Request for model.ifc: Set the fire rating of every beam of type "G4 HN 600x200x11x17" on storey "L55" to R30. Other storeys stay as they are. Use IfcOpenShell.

First a look at what the model holds.

```python
import ifcopenshell
import ifcopenshell.util.element

model = ifcopenshell.open("model.ifc")
print(model.schema)
storey = next(s for s in model.by_type("IfcBuildingStorey") if s.Name == "L55")
beams = [e for e in ifcopenshell.util.element.get_decomposition(storey) if e.is_a("IfcBeam")]
seen = {}
for e in beams:
    element_type = ifcopenshell.util.element.get_type(e)
    key = (element_type.Name if element_type != e and element_type else None, ifcopenshell.util.element.get_pset(e, "Pset_BeamCommon", "FireRating"))
    seen[key] = seen.get(key, 0) + 1
for (name, value), count in sorted(seen.items(), key=str):
    print(count, "x", name, "|", value)
```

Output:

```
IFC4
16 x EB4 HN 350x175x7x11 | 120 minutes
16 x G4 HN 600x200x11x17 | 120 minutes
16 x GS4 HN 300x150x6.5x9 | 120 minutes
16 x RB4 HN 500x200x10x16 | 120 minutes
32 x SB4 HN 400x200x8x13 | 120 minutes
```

```python
import ifcopenshell
import ifcopenshell.api.pset
import ifcopenshell.util.element

model = ifcopenshell.open("model.ifc")

storey = next(s for s in model.by_type("IfcBuildingStorey") if s.Name == "L55")
beams = [e for e in ifcopenshell.util.element.get_decomposition(storey) if e.is_a("IfcBeam")]

count = 0
for e in beams:
    element_type = ifcopenshell.util.element.get_type(e)
    if element_type in (None, e) or element_type.Name != "G4 HN 600x200x11x17":
        continue
    found = ifcopenshell.util.element.get_pset(e, "Pset_BeamCommon", should_inherit=False)
    if found:
        pset = model.by_id(found["id"])
        if len(ifcopenshell.util.element.get_elements_by_pset(pset)) > 1:
            pset = ifcopenshell.api.pset.unshare_pset(model, products=[e], pset=pset)[0]
    else:
        pset = ifcopenshell.api.pset.add_pset(model, product=e, name="Pset_BeamCommon")
    ifcopenshell.api.pset.edit_pset(model, pset=pset, properties={"FireRating": "R30"})
    count += 1

print(count, "beams updated")

model.write("model-out.ifc")
```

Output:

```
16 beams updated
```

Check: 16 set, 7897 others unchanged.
